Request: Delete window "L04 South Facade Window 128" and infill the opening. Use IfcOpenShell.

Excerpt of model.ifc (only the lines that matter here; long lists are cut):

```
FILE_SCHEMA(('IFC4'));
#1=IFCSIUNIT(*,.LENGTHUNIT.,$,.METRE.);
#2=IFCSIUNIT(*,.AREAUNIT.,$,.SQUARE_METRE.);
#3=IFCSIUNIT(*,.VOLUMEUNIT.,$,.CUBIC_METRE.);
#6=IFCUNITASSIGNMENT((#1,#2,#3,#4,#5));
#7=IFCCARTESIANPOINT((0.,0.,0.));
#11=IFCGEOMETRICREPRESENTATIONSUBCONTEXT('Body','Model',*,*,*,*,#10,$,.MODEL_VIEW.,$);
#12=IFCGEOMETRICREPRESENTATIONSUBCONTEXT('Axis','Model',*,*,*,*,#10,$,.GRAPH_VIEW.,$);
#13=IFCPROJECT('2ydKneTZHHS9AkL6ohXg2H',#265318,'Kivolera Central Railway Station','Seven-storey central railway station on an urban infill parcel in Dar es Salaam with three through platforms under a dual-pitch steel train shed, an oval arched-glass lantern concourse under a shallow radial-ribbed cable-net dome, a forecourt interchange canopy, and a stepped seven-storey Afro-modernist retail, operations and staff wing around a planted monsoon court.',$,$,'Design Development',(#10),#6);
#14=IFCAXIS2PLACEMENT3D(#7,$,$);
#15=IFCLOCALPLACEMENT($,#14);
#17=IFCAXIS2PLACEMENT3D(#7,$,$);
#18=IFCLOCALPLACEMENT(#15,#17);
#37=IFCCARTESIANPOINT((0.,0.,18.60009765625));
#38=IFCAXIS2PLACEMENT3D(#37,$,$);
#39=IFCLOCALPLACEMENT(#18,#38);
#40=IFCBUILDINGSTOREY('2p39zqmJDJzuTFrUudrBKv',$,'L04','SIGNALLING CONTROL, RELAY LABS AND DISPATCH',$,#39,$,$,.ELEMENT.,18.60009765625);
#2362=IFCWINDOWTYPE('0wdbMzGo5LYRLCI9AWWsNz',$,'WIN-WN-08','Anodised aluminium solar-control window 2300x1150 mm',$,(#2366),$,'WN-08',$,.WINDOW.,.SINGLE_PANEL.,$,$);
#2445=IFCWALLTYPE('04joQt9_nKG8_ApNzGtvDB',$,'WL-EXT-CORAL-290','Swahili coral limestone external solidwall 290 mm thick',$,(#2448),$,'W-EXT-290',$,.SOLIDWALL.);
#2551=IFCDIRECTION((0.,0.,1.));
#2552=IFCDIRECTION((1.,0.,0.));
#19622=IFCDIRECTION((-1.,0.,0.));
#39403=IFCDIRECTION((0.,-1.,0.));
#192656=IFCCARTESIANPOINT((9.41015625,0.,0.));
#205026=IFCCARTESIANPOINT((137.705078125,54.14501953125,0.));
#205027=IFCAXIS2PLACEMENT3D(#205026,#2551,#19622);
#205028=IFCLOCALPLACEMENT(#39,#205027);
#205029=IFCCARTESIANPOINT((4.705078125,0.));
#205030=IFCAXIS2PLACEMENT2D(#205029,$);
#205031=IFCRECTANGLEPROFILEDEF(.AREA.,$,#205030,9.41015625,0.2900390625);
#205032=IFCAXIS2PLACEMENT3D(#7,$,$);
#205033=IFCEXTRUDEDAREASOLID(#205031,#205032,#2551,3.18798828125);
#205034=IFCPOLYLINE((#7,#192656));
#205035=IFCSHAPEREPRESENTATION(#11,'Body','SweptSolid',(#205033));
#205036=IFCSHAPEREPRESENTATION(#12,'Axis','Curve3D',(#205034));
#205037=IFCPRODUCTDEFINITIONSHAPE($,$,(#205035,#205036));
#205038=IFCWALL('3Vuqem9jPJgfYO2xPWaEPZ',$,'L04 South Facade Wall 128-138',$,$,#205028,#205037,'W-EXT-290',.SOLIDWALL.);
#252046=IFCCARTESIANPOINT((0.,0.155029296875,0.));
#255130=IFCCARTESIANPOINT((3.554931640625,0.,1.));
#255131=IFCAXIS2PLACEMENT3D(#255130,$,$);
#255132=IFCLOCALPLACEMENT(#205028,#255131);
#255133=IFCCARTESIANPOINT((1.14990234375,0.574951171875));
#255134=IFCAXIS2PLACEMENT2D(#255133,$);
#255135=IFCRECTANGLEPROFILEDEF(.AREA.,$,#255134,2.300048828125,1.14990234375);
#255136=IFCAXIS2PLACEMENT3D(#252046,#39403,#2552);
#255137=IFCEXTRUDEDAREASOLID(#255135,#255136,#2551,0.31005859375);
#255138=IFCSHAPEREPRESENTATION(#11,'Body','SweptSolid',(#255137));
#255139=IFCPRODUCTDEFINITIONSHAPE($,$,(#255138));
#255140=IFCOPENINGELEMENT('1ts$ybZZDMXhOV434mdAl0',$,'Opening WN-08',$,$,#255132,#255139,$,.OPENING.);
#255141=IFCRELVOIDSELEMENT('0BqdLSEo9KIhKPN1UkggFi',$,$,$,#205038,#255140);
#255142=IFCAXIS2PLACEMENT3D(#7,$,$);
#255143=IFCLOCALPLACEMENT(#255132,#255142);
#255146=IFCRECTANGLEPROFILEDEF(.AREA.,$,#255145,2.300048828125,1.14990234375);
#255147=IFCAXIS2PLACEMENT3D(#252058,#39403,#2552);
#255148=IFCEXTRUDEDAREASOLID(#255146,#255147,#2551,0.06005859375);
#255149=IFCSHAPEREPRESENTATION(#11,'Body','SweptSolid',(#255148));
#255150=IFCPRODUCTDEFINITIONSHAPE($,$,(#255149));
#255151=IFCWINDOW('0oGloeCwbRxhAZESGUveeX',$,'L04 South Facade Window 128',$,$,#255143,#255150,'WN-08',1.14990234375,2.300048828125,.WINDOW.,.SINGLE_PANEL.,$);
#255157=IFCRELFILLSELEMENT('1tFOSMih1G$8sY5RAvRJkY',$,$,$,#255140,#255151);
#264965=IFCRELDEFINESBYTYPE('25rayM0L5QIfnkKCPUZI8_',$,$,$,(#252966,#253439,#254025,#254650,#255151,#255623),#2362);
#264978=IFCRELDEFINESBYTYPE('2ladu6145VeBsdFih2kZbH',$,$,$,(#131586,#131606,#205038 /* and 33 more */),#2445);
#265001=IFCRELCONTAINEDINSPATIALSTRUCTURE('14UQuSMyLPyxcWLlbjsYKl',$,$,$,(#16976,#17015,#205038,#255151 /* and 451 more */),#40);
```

```python
import ifcopenshell
import ifcopenshell.api.feature
import ifcopenshell.api.root
import ifcopenshell.geom
import ifcopenshell.util.shape

model = ifcopenshell.open("model.ifc")
settings = ifcopenshell.geom.settings()


def volume(element):
    """Net volume in cubic metres, openings subtracted."""
    shape = ifcopenshell.geom.create_shape(settings, element)
    return ifcopenshell.util.shape.get_volume(shape.geometry)


window = model.by_guid("0oGloeCwbRxhAZESGUveeX")
opening = window.FillsVoids[0].RelatingOpeningElement
wall = opening.VoidsElements[0].RelatingBuildingElement
before = volume(wall)

ifcopenshell.api.root.remove_product(model, product=window)
ifcopenshell.api.feature.remove_feature(model, feature=opening)

after = volume(wall)

print(f"wall volume {before:.3f} -> {after:.3f} m3")

model.write("model-out.ifc")
```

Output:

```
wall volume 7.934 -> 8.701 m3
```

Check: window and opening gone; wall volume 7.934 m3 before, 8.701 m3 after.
